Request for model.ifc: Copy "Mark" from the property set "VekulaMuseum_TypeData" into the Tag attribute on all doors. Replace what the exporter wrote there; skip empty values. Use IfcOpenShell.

First a look at what the model holds.

```python
import ifcopenshell
import ifcopenshell.util.element

model = ifcopenshell.open("model.ifc")
print(model.schema)
doors = model.by_type("IfcDoor")
print(len(doors), "doors")
for e in doors[:8]:
    source = ifcopenshell.util.element.get_pset(e, "VekulaMuseum_TypeData", "Mark")
    target = e.Tag
    print(e.id(), repr(source), repr(target), sep=" | ")
```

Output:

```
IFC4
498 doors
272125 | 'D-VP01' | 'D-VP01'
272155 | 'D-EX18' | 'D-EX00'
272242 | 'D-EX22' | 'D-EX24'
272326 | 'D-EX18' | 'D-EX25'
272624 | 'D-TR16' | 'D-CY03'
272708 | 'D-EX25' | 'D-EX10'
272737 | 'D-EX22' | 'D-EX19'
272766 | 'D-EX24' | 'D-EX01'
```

```python
import ifcopenshell
import ifcopenshell.util.element

model = ifcopenshell.open("model.ifc")

count = 0
for e in model.by_type("IfcDoor"):
    value = ifcopenshell.util.element.get_pset(e, "VekulaMuseum_TypeData", "Mark")
    current = e.Tag
    if not value or not value.strip() or current == value:
        continue
    e.Tag = value
    count += 1

print(count, "doors updated")

model.write("model_updated.ifc")
```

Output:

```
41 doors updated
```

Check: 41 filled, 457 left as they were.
